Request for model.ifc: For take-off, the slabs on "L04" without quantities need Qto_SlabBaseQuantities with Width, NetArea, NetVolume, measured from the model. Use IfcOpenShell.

First a look at what the model holds.

```python
import ifcopenshell
import ifcopenshell.util.element
import ifcopenshell.util.unit

model = ifcopenshell.open("model.ifc")
print(model.schema)
for unit_type in ("LENGTHUNIT", "AREAUNIT", "VOLUMEUNIT"):
    print(unit_type, ifcopenshell.util.unit.calculate_unit_scale(model, unit_type))
storey = next(s for s in model.by_type("IfcBuildingStorey") if s.Name == "L04")
slabs = [e for e in ifcopenshell.util.element.get_decomposition(storey) if e.is_a("IfcSlab")]
for e in sorted(slabs, key=lambda e: e.id()):
    print(e.id(), e.is_a(), e.Name, list(ifcopenshell.util.element.get_psets(e, qtos_only=True)), sep=" | ")
```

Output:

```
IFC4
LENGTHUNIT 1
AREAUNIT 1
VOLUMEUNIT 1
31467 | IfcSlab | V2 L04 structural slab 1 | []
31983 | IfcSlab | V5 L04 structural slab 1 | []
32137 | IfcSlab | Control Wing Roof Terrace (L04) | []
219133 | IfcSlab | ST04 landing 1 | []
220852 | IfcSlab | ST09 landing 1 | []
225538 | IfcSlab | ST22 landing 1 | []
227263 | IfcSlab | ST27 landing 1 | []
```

```python
import ifcopenshell
import ifcopenshell.api.pset
import ifcopenshell.geom
import ifcopenshell.util.element
import ifcopenshell.util.shape
import ifcopenshell.util.unit

model = ifcopenshell.open("model.ifc")
unit_scale = ifcopenshell.util.unit.calculate_unit_scale(model)
area_scale = ifcopenshell.util.unit.calculate_unit_scale(model, "AREAUNIT")
volume_scale = ifcopenshell.util.unit.calculate_unit_scale(model, "VOLUMEUNIT")
settings = ifcopenshell.geom.settings()

storey = next(s for s in model.by_type("IfcBuildingStorey") if s.Name == "L04")
slabs = [e for e in ifcopenshell.util.element.get_decomposition(storey) if e.is_a("IfcSlab")]

for e in sorted(slabs, key=lambda e: e.id()):
    if ifcopenshell.util.element.get_psets(e, qtos_only=True, should_inherit=False):
        continue
    # Geometry comes back in metres, in the element's own axes.
    shape = ifcopenshell.geom.create_shape(settings, e)
    values = {
        "Width": ifcopenshell.util.shape.get_z(shape.geometry) / unit_scale,
        "NetArea": ifcopenshell.util.shape.get_footprint_area(shape.geometry) / area_scale,
        "NetVolume": ifcopenshell.util.shape.get_volume(shape.geometry) / volume_scale,
    }
    qto = ifcopenshell.api.pset.add_qto(model, product=e, name="Qto_SlabBaseQuantities")
    ifcopenshell.api.pset.edit_qto(model, qto=qto, properties=values)
    print(e.id(), {k: round(v, 3) for k, v in values.items()})

model.write("model_v2.ifc")
```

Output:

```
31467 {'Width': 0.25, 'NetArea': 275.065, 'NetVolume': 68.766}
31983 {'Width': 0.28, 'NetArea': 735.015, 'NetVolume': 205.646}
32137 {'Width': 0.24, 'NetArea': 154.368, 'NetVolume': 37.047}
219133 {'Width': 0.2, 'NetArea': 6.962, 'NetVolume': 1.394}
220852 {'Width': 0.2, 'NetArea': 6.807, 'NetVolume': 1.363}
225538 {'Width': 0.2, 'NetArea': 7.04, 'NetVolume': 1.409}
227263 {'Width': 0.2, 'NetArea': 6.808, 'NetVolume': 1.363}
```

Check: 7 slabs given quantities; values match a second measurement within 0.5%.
